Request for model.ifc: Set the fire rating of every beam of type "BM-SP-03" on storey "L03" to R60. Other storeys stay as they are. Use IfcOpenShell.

First a look at what the model holds.

```python
import ifcopenshell
import ifcopenshell.util.element

model = ifcopenshell.open("model.ifc")
print(model.schema)
storey = next(s for s in model.by_type("IfcBuildingStorey") if s.Name == "L03")
beams = [e for e in ifcopenshell.util.element.get_decomposition(storey) if e.is_a("IfcBeam")]
seen = {}
for e in beams:
    element_type = ifcopenshell.util.element.get_type(e)
    key = (element_type.Name if element_type != e and element_type else None, ifcopenshell.util.element.get_pset(e, "Pset_BeamCommon", "FireRating"))
    seen[key] = seen.get(key, 0) + 1
for (name, value), count in sorted(seen.items(), key=str):
    print(count, "x", name, "|", value)
```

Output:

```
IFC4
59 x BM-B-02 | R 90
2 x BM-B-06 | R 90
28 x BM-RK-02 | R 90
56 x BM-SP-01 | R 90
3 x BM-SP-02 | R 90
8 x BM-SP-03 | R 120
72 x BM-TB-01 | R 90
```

```python
import ifcopenshell
import ifcopenshell.api.pset
import ifcopenshell.util.element

model = ifcopenshell.open("model.ifc")

storey = next(s for s in model.by_type("IfcBuildingStorey") if s.Name == "L03")
beams = [e for e in ifcopenshell.util.element.get_decomposition(storey) if e.is_a("IfcBeam")]

count = 0
for e in beams:
    element_type = ifcopenshell.util.element.get_type(e)
    if element_type in (None, e) or element_type.Name != "BM-SP-03":
        continue
    # add_pset returns the element's existing set when there is one.
    pset = ifcopenshell.api.pset.add_pset(model, product=e, name="Pset_BeamCommon")
    ifcopenshell.api.pset.edit_pset(model, pset=pset, properties={"FireRating": "R60"})
    count += 1

print(count, "beams updated")

model.write("model-out.ifc")
```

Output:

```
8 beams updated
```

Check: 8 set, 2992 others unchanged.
